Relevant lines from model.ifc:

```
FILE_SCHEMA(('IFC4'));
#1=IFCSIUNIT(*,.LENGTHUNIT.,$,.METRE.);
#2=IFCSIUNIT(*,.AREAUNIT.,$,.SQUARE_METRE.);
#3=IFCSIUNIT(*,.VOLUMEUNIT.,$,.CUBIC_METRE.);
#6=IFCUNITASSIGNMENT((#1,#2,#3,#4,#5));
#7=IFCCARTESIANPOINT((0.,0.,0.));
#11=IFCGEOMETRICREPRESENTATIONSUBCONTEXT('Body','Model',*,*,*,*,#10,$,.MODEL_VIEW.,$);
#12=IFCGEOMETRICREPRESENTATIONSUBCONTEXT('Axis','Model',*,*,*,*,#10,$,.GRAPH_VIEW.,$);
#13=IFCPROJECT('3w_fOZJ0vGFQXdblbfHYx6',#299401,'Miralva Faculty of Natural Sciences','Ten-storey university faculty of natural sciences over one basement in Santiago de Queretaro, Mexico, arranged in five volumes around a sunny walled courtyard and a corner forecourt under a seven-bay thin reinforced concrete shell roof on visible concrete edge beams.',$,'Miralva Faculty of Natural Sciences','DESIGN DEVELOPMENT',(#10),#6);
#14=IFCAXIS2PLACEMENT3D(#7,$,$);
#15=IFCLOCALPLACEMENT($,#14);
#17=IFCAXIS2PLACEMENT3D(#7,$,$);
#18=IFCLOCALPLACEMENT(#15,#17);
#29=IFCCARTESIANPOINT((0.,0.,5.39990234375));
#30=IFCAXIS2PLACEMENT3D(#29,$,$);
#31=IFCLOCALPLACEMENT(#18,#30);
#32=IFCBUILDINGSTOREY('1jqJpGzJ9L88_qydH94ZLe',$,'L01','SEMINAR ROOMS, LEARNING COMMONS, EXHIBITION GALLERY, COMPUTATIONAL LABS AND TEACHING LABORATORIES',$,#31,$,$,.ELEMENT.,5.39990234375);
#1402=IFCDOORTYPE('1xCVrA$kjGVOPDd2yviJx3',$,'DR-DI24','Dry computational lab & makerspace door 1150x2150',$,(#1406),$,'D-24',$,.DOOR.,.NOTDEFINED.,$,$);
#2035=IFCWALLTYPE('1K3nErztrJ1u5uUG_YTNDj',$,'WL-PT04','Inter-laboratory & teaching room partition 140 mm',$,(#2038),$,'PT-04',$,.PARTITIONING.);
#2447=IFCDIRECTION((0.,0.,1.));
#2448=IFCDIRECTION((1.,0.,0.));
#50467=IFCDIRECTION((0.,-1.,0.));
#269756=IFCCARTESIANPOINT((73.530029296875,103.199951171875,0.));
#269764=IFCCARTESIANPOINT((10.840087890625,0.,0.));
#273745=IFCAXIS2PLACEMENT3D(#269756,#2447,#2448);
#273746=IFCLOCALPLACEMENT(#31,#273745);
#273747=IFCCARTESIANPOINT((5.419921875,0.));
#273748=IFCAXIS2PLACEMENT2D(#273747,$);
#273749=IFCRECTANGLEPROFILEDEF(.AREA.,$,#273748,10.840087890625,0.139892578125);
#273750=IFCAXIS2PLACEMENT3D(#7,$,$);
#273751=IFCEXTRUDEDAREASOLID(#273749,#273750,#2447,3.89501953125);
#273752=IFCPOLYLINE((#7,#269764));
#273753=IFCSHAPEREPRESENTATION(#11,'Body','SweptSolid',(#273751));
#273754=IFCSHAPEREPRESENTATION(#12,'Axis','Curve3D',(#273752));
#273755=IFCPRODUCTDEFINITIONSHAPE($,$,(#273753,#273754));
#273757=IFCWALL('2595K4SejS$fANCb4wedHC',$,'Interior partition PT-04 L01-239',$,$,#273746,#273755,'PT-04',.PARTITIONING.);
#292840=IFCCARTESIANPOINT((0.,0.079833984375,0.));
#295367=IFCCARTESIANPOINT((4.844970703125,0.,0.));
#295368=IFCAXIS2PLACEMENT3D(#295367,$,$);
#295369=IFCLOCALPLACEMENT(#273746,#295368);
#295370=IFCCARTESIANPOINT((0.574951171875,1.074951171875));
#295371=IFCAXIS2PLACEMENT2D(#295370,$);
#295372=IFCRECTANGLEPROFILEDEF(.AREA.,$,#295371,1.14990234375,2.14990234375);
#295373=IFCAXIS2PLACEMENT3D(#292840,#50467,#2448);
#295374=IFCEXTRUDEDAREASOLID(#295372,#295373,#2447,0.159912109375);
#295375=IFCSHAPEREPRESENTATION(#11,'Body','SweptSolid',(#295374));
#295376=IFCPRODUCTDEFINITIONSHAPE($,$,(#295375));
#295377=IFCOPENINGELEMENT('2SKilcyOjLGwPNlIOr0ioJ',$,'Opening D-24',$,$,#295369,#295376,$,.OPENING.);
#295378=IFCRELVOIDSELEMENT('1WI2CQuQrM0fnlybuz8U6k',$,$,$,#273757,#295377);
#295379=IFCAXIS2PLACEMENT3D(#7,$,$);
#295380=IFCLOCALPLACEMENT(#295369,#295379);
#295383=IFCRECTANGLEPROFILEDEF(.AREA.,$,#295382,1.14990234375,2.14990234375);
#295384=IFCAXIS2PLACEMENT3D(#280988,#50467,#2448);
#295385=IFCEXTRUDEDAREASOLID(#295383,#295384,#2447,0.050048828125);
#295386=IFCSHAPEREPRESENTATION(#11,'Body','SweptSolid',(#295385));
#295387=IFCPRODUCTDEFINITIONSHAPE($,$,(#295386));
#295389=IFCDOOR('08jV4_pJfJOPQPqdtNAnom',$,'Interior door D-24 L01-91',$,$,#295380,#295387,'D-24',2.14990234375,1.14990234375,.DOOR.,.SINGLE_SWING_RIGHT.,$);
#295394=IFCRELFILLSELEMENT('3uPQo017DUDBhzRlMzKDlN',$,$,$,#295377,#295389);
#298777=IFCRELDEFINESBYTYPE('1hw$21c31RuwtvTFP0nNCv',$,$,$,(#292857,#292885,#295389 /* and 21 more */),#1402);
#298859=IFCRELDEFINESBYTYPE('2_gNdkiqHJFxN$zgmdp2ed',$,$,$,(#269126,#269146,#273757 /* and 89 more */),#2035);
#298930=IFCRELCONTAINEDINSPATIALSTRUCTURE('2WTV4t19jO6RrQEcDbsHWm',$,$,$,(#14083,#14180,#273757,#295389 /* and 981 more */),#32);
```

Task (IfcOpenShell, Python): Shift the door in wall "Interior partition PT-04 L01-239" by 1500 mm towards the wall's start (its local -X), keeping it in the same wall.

```python
import ifcopenshell
import ifcopenshell.api.geometry
import ifcopenshell.util.placement
import ifcopenshell.util.unit

model = ifcopenshell.open("model.ifc")
unit_scale = ifcopenshell.util.unit.calculate_unit_scale(model)

door = model.by_guid("08jV4_pJfJOPQPqdtNAnom")
opening = door.FillsVoids[0].RelatingOpeningElement
wall = opening.VoidsElements[0].RelatingBuildingElement

wall_matrix = ifcopenshell.util.placement.get_local_placement(wall.ObjectPlacement)
shift = wall_matrix[:3, 0] * -1.5 / unit_scale
before = ifcopenshell.util.placement.get_local_placement(door.ObjectPlacement)[:3, 3].copy()

# The door is placed relative to its opening, so it follows when the opening moves.
matrix = ifcopenshell.util.placement.get_local_placement(opening.ObjectPlacement)
matrix[:3, 3] += shift
ifcopenshell.api.geometry.edit_object_placement(
    model, product=opening, matrix=matrix, is_si=False, should_transform_children=True
)

after = ifcopenshell.util.placement.get_local_placement(door.ObjectPlacement)[:3, 3]
print("door moved by", (after - before).round(3) + 0.0)

model.write("model_updated.ifc")
```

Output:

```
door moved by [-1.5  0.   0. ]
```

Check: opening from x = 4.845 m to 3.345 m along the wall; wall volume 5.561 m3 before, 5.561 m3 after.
